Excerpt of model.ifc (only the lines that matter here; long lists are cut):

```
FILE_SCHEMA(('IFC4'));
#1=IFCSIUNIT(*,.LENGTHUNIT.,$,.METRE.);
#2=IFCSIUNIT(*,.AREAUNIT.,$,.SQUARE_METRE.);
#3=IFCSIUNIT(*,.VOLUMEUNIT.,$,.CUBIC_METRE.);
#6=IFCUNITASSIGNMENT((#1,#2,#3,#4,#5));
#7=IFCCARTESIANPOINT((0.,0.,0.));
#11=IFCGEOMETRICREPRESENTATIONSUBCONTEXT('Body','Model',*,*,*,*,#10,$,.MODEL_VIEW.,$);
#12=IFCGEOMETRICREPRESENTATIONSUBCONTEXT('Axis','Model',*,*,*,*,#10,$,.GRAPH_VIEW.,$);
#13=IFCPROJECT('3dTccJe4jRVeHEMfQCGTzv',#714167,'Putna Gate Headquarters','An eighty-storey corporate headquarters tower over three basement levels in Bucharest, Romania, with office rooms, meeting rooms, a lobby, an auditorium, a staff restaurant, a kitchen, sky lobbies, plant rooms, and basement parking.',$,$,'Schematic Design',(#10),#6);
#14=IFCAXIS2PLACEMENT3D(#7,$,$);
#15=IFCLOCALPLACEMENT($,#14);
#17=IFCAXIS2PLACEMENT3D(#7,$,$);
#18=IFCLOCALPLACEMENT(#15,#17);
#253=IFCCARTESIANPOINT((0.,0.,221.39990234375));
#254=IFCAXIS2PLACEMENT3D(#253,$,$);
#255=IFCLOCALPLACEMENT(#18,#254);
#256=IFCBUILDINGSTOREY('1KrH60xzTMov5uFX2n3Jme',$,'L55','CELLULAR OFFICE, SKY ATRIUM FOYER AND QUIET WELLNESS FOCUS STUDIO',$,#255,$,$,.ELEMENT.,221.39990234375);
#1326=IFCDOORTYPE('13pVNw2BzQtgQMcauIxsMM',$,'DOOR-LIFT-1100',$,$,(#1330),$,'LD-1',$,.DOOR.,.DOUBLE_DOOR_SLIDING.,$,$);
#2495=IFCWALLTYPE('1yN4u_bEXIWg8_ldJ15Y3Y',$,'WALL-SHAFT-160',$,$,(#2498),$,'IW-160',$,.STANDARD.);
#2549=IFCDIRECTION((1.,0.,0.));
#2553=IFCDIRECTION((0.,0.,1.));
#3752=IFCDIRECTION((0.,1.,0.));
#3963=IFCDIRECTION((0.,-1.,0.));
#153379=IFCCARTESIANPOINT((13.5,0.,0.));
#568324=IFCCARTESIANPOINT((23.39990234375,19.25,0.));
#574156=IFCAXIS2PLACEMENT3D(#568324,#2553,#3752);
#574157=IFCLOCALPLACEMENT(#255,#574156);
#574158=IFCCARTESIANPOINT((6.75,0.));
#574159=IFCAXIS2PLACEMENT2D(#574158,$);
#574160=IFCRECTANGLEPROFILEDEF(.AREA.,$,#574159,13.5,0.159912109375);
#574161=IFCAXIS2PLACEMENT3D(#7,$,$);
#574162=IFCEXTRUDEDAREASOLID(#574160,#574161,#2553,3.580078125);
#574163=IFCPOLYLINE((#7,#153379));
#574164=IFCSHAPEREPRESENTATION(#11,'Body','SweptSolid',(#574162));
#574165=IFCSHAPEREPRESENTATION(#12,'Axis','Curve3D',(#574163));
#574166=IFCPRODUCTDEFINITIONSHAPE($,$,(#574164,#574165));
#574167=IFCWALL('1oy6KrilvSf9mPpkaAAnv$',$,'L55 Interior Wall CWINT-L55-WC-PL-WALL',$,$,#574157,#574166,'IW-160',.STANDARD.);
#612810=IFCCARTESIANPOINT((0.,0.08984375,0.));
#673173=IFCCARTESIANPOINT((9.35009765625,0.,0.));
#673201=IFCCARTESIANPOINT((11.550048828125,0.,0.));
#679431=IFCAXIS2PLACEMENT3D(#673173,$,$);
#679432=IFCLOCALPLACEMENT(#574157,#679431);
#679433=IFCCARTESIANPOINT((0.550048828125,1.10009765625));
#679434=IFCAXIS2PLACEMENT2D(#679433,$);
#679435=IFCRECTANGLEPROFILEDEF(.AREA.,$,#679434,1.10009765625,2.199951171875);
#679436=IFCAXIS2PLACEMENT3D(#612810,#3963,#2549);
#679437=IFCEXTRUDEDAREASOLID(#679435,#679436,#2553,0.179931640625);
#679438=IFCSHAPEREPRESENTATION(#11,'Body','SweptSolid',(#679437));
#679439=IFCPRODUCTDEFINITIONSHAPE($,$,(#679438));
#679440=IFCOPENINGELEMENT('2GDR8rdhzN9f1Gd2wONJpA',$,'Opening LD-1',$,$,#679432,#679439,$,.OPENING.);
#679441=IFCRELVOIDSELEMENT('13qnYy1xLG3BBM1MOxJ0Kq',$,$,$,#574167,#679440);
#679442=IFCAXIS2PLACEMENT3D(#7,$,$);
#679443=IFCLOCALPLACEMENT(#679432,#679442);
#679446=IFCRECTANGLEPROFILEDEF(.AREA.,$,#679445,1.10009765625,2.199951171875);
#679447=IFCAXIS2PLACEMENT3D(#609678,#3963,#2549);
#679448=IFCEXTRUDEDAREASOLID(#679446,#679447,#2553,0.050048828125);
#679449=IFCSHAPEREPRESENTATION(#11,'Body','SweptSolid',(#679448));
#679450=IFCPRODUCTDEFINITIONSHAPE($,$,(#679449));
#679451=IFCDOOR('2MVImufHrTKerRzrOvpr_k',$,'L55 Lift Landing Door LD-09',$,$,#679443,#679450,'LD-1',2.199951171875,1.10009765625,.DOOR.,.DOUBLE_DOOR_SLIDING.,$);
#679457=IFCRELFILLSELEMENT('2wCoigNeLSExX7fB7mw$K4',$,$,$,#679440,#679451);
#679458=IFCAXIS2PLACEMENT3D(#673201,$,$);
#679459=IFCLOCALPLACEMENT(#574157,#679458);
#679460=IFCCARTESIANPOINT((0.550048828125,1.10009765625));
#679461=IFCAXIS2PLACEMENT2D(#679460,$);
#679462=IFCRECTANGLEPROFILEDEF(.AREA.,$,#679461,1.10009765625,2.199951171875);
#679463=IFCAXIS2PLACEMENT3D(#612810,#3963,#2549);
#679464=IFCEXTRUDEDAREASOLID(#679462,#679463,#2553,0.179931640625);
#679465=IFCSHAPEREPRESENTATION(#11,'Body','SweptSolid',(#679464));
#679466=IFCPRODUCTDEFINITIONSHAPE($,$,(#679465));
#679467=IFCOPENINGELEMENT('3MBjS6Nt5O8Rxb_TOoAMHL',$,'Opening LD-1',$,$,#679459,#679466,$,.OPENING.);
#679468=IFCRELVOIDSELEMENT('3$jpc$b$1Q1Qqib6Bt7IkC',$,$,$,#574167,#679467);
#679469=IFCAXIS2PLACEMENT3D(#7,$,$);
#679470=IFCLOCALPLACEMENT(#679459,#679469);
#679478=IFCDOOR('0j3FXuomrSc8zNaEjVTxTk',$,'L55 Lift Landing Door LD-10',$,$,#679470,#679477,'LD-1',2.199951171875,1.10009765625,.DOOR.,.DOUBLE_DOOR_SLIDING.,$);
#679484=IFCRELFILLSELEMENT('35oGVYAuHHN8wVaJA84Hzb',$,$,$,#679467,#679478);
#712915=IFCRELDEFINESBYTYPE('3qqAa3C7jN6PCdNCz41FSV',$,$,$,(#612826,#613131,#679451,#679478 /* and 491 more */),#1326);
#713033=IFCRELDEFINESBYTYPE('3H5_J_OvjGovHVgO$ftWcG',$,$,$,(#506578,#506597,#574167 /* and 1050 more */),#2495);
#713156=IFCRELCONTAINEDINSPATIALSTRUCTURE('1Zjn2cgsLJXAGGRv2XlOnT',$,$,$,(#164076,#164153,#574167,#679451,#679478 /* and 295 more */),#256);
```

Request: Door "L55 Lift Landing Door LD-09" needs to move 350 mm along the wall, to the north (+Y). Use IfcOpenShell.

```python
import ifcopenshell
import ifcopenshell.api.geometry
import ifcopenshell.util.placement
import ifcopenshell.util.unit

model = ifcopenshell.open("model.ifc")
unit_scale = ifcopenshell.util.unit.calculate_unit_scale(model)

door = model.by_guid("2MVImufHrTKerRzrOvpr_k")
opening = door.FillsVoids[0].RelatingOpeningElement
wall = opening.VoidsElements[0].RelatingBuildingElement

wall_matrix = ifcopenshell.util.placement.get_local_placement(wall.ObjectPlacement)
shift = wall_matrix[:3, 0] * 0.35 / unit_scale
before = ifcopenshell.util.placement.get_local_placement(door.ObjectPlacement)[:3, 3].copy()

# The door is placed relative to its opening, so it follows when the opening moves.
matrix = ifcopenshell.util.placement.get_local_placement(opening.ObjectPlacement)
matrix[:3, 3] += shift
ifcopenshell.api.geometry.edit_object_placement(
    model, product=opening, matrix=matrix, is_si=False, should_transform_children=True
)

after = ifcopenshell.util.placement.get_local_placement(door.ObjectPlacement)[:3, 3]
print("door moved by", (after - before).round(3) + 0.0)

model.write("model_updated.ifc")
```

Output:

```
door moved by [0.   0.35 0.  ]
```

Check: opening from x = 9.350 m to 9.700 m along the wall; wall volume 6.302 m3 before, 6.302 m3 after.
